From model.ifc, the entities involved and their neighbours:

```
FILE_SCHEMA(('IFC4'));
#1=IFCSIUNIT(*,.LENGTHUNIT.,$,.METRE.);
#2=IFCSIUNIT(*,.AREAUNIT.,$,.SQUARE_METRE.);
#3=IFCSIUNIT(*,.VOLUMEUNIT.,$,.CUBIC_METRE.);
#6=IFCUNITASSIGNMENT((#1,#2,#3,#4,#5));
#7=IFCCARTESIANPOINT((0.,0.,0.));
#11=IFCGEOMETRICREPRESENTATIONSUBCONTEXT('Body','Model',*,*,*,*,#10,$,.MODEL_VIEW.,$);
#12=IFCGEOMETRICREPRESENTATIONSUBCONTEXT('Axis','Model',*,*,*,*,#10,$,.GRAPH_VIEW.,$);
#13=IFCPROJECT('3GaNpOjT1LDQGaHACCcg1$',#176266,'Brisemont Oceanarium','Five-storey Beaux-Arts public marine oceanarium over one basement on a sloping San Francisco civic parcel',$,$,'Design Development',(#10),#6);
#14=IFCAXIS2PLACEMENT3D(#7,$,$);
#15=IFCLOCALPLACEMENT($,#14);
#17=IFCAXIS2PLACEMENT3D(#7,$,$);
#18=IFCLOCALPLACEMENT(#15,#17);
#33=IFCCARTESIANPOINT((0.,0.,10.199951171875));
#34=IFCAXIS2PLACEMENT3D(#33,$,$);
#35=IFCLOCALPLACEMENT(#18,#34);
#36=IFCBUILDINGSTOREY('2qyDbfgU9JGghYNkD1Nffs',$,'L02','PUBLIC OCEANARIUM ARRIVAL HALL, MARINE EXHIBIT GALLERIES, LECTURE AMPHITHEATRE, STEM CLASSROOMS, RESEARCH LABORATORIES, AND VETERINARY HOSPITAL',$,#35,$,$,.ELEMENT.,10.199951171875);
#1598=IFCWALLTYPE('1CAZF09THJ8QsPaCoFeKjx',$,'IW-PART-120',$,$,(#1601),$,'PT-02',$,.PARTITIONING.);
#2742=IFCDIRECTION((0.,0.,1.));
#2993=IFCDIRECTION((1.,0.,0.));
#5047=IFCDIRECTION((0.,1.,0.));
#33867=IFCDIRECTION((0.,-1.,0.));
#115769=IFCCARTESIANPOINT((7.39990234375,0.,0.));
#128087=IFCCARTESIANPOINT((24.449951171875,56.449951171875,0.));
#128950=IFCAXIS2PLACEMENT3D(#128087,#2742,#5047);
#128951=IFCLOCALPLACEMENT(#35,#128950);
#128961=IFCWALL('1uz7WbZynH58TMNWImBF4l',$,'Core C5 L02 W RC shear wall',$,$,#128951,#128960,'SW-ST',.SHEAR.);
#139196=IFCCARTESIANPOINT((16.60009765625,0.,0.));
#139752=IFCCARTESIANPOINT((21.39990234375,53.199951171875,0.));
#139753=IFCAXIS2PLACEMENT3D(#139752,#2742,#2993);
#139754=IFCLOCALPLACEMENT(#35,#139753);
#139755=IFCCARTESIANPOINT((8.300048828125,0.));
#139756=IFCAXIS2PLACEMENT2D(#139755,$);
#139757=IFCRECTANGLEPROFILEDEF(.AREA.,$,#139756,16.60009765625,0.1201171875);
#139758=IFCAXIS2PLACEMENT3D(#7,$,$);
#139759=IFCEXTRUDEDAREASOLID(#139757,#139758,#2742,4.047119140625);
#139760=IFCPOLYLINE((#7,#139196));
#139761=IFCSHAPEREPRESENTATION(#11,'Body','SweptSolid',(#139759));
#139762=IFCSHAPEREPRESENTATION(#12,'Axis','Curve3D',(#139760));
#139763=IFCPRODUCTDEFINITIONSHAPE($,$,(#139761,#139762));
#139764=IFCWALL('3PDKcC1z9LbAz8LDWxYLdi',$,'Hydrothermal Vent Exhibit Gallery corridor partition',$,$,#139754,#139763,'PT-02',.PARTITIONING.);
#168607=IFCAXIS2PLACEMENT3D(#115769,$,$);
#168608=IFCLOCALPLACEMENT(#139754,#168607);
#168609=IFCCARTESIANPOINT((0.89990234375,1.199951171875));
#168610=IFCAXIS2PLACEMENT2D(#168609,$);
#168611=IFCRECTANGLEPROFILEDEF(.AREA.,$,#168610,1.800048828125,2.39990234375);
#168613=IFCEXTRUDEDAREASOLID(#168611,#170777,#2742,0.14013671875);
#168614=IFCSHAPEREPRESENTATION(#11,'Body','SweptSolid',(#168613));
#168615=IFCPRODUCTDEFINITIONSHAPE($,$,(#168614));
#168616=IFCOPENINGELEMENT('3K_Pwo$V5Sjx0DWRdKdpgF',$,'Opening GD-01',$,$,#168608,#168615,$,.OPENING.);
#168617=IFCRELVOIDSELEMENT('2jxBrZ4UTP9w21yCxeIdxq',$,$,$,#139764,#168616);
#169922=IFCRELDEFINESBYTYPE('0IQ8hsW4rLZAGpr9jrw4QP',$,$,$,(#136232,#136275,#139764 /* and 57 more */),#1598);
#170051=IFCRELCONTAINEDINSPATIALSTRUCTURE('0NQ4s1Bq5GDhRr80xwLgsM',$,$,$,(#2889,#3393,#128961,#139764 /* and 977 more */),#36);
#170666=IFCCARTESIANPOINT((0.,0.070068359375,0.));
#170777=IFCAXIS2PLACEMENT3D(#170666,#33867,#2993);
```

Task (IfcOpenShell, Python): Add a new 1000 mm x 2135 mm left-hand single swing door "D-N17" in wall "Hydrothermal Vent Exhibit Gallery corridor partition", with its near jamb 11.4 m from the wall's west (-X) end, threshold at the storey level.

```python
import numpy as np
import ifcopenshell
import ifcopenshell.api.feature
import ifcopenshell.api.geometry
import ifcopenshell.api.root
import ifcopenshell.api.spatial
import ifcopenshell.geom
import ifcopenshell.util.element
import ifcopenshell.util.placement
import ifcopenshell.util.representation
import ifcopenshell.util.shape
import ifcopenshell.util.unit

model = ifcopenshell.open("model.ifc")
unit_scale = ifcopenshell.util.unit.calculate_unit_scale(model)
settings = ifcopenshell.geom.settings()


def volume(element):
    """Net volume in cubic metres, openings subtracted."""
    shape = ifcopenshell.geom.create_shape(settings, element)
    return ifcopenshell.util.shape.get_volume(shape.geometry)


wall = model.by_id(139764)
storey = ifcopenshell.util.element.get_container(wall, ifc_class="IfcBuildingStorey")
context = ifcopenshell.util.representation.get_context(model, "Model", "Body", "MODEL_VIEW")
before = volume(wall)

width, height, from_end, sill = 1, 2.135, 11.4, 0.0  # metres

# The wall runs along its own X axis, and the end named is its -X end.
wall_shape = ifcopenshell.geom.create_shape(settings, wall)
x, y, z = ifcopenshell.util.shape.get_vertices(wall_shape.geometry).T
start = x.min() + from_end
face, thickness = float(y.min()), float(y.max() - y.min())
wall_matrix = ifcopenshell.util.placement.get_local_placement(wall.ObjectPlacement)
level = ifcopenshell.util.placement.get_local_placement(storey.ObjectPlacement)[2, 3]


def in_wall(x, y):
    """Placement at x, y metres in the wall's axes, at sill height."""
    matrix = wall_matrix.copy()
    matrix[:, 3] = wall_matrix @ np.array([x / unit_scale, y / unit_scale, 0.0, 1.0])
    matrix[2, 3] = level + sill / unit_scale
    return matrix


# Opening: a box that overshoots both wall faces by 50 mm.
opening = ifcopenshell.api.root.create_entity(model, ifc_class="IfcOpeningElement", predefined_type="OPENING")
box = ifcopenshell.api.geometry.add_wall_representation(
    model, context=context, length=width, height=height, thickness=thickness + 0.1
)
ifcopenshell.api.geometry.assign_representation(model, product=opening, representation=box)
ifcopenshell.api.geometry.edit_object_placement(model, product=opening, matrix=in_wall(start, face - 0.05), is_si=False)
ifcopenshell.api.feature.add_feature(model, feature=opening, element=wall)

door = ifcopenshell.api.root.create_entity(model, ifc_class="IfcDoor", name="D-N17", predefined_type="DOOR")
door.OverallWidth, door.OverallHeight = width / unit_scale, height / unit_scale
door.OperationType = "SINGLE_SWING_LEFT"
body = ifcopenshell.api.geometry.add_door_representation(
    model,
    context=context,
    overall_width=door.OverallWidth,
    overall_height=door.OverallHeight,
    operation_type="SINGLE_SWING_LEFT",
    lining_properties={"LiningDepth": thickness / unit_scale, "ThresholdDepth": thickness / unit_scale},
)
ifcopenshell.api.geometry.assign_representation(model, product=door, representation=body)
ifcopenshell.api.spatial.assign_container(model, products=[door], relating_structure=storey)
ifcopenshell.api.feature.add_filling(model, opening=opening, element=door)

# The lining spans the wall, so the door starts at the wall face.
ifcopenshell.api.geometry.edit_object_placement(model, product=door, matrix=in_wall(start, face), is_si=False)

after = volume(wall)

print(f"wall volume {before:.3f} -> {after:.3f} m3")

model.write("model-out.ifc")
```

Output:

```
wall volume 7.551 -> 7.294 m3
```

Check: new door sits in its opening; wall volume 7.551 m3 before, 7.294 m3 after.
